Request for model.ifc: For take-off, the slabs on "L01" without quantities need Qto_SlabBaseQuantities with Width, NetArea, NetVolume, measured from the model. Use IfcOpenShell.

First a look at what the model holds.

```python
import ifcopenshell
import ifcopenshell.util.element
import ifcopenshell.util.unit

model = ifcopenshell.open("model.ifc")
print(model.schema)
for unit_type in ("LENGTHUNIT", "AREAUNIT", "VOLUMEUNIT"):
    print(unit_type, ifcopenshell.util.unit.calculate_unit_scale(model, unit_type))
storey = next(s for s in model.by_type("IfcBuildingStorey") if s.Name == "L01")
slabs = [e for e in ifcopenshell.util.element.get_decomposition(storey) if e.is_a("IfcSlab")]
for e in sorted(slabs, key=lambda e: e.id()):
    print(e.id(), e.is_a(), e.Name, list(ifcopenshell.util.element.get_psets(e, qtos_only=True)), sep=" | ")
```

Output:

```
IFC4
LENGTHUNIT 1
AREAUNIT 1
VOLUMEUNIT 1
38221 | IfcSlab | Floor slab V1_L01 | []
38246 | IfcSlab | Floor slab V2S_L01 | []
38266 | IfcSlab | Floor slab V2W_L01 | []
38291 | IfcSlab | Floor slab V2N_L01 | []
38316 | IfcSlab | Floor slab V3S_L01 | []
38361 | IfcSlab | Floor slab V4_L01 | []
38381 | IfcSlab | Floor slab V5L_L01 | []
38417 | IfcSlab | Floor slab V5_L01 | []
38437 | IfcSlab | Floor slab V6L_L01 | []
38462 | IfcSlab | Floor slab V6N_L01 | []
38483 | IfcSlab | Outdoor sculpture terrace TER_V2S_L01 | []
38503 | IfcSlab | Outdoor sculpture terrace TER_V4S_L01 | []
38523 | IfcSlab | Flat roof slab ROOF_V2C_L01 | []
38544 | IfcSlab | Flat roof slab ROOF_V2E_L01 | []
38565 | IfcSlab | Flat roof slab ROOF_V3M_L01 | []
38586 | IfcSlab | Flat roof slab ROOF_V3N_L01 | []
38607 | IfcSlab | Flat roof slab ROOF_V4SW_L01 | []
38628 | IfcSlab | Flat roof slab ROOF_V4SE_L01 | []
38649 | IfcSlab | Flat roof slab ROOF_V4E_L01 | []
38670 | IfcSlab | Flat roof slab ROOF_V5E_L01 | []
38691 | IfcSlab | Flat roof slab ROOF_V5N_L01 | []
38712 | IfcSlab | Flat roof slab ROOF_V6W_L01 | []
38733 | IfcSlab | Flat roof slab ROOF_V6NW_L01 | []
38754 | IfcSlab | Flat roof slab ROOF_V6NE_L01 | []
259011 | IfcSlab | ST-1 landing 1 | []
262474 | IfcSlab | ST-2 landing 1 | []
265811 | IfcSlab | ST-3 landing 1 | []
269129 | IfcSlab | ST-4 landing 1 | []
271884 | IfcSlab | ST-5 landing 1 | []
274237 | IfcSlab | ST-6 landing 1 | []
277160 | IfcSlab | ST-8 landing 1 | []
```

```python
import ifcopenshell
import ifcopenshell.api.pset
import ifcopenshell.geom
import ifcopenshell.util.element
import ifcopenshell.util.shape
import ifcopenshell.util.unit

model = ifcopenshell.open("model.ifc")
unit_scale = ifcopenshell.util.unit.calculate_unit_scale(model)
area_scale = ifcopenshell.util.unit.calculate_unit_scale(model, "AREAUNIT")
volume_scale = ifcopenshell.util.unit.calculate_unit_scale(model, "VOLUMEUNIT")
settings = ifcopenshell.geom.settings()

storey = next(s for s in model.by_type("IfcBuildingStorey") if s.Name == "L01")
slabs = [e for e in ifcopenshell.util.element.get_decomposition(storey) if e.is_a("IfcSlab")]

for e in sorted(slabs, key=lambda e: e.id()):
    if ifcopenshell.util.element.get_psets(e, qtos_only=True, should_inherit=False):
        continue
    # Geometry comes back in metres, in the element's own axes.
    shape = ifcopenshell.geom.create_shape(settings, e)
    values = {
        "Width": ifcopenshell.util.shape.get_z(shape.geometry) / unit_scale,
        "NetArea": ifcopenshell.util.shape.get_footprint_area(shape.geometry) / area_scale,
        "NetVolume": ifcopenshell.util.shape.get_volume(shape.geometry) / volume_scale,
    }
    qto = ifcopenshell.api.pset.add_qto(model, product=e, name="Qto_SlabBaseQuantities")
    ifcopenshell.api.pset.edit_qto(model, qto=qto, properties=values)
    print(e.id(), {k: round(v, 3) for k, v in values.items()})

model.write("model-out.ifc")
```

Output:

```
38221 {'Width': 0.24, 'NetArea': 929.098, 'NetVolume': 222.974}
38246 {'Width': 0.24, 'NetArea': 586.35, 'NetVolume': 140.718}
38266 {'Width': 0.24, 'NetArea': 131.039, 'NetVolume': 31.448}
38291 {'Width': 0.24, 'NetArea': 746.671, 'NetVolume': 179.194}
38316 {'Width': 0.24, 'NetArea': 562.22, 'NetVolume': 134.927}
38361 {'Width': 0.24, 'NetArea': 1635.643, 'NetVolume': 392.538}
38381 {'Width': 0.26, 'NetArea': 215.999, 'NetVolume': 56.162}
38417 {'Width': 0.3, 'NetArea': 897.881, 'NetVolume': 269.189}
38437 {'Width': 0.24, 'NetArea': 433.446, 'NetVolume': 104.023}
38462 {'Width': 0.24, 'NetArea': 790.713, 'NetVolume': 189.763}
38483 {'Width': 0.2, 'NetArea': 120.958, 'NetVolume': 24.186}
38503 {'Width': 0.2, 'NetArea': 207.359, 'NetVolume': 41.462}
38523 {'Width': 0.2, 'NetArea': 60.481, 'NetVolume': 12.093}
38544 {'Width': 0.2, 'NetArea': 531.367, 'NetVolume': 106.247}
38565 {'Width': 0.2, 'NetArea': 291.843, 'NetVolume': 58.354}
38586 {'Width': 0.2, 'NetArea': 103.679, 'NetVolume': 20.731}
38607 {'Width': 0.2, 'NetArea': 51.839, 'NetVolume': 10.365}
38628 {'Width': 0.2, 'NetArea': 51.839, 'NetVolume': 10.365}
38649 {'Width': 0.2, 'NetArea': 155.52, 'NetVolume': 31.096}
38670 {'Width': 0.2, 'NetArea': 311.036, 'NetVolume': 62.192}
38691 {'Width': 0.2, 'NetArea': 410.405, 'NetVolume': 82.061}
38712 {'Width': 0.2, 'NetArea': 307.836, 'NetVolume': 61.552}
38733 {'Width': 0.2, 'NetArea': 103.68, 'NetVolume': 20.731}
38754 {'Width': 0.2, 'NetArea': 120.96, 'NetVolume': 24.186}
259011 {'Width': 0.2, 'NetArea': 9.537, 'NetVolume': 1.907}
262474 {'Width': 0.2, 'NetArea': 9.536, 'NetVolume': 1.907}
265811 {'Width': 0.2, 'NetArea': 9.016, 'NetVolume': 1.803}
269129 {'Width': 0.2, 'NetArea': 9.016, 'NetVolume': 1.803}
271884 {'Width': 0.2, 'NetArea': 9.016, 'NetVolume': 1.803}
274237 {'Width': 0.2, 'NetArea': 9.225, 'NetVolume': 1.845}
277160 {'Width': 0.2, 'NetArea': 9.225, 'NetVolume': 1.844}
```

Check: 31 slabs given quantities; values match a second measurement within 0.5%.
